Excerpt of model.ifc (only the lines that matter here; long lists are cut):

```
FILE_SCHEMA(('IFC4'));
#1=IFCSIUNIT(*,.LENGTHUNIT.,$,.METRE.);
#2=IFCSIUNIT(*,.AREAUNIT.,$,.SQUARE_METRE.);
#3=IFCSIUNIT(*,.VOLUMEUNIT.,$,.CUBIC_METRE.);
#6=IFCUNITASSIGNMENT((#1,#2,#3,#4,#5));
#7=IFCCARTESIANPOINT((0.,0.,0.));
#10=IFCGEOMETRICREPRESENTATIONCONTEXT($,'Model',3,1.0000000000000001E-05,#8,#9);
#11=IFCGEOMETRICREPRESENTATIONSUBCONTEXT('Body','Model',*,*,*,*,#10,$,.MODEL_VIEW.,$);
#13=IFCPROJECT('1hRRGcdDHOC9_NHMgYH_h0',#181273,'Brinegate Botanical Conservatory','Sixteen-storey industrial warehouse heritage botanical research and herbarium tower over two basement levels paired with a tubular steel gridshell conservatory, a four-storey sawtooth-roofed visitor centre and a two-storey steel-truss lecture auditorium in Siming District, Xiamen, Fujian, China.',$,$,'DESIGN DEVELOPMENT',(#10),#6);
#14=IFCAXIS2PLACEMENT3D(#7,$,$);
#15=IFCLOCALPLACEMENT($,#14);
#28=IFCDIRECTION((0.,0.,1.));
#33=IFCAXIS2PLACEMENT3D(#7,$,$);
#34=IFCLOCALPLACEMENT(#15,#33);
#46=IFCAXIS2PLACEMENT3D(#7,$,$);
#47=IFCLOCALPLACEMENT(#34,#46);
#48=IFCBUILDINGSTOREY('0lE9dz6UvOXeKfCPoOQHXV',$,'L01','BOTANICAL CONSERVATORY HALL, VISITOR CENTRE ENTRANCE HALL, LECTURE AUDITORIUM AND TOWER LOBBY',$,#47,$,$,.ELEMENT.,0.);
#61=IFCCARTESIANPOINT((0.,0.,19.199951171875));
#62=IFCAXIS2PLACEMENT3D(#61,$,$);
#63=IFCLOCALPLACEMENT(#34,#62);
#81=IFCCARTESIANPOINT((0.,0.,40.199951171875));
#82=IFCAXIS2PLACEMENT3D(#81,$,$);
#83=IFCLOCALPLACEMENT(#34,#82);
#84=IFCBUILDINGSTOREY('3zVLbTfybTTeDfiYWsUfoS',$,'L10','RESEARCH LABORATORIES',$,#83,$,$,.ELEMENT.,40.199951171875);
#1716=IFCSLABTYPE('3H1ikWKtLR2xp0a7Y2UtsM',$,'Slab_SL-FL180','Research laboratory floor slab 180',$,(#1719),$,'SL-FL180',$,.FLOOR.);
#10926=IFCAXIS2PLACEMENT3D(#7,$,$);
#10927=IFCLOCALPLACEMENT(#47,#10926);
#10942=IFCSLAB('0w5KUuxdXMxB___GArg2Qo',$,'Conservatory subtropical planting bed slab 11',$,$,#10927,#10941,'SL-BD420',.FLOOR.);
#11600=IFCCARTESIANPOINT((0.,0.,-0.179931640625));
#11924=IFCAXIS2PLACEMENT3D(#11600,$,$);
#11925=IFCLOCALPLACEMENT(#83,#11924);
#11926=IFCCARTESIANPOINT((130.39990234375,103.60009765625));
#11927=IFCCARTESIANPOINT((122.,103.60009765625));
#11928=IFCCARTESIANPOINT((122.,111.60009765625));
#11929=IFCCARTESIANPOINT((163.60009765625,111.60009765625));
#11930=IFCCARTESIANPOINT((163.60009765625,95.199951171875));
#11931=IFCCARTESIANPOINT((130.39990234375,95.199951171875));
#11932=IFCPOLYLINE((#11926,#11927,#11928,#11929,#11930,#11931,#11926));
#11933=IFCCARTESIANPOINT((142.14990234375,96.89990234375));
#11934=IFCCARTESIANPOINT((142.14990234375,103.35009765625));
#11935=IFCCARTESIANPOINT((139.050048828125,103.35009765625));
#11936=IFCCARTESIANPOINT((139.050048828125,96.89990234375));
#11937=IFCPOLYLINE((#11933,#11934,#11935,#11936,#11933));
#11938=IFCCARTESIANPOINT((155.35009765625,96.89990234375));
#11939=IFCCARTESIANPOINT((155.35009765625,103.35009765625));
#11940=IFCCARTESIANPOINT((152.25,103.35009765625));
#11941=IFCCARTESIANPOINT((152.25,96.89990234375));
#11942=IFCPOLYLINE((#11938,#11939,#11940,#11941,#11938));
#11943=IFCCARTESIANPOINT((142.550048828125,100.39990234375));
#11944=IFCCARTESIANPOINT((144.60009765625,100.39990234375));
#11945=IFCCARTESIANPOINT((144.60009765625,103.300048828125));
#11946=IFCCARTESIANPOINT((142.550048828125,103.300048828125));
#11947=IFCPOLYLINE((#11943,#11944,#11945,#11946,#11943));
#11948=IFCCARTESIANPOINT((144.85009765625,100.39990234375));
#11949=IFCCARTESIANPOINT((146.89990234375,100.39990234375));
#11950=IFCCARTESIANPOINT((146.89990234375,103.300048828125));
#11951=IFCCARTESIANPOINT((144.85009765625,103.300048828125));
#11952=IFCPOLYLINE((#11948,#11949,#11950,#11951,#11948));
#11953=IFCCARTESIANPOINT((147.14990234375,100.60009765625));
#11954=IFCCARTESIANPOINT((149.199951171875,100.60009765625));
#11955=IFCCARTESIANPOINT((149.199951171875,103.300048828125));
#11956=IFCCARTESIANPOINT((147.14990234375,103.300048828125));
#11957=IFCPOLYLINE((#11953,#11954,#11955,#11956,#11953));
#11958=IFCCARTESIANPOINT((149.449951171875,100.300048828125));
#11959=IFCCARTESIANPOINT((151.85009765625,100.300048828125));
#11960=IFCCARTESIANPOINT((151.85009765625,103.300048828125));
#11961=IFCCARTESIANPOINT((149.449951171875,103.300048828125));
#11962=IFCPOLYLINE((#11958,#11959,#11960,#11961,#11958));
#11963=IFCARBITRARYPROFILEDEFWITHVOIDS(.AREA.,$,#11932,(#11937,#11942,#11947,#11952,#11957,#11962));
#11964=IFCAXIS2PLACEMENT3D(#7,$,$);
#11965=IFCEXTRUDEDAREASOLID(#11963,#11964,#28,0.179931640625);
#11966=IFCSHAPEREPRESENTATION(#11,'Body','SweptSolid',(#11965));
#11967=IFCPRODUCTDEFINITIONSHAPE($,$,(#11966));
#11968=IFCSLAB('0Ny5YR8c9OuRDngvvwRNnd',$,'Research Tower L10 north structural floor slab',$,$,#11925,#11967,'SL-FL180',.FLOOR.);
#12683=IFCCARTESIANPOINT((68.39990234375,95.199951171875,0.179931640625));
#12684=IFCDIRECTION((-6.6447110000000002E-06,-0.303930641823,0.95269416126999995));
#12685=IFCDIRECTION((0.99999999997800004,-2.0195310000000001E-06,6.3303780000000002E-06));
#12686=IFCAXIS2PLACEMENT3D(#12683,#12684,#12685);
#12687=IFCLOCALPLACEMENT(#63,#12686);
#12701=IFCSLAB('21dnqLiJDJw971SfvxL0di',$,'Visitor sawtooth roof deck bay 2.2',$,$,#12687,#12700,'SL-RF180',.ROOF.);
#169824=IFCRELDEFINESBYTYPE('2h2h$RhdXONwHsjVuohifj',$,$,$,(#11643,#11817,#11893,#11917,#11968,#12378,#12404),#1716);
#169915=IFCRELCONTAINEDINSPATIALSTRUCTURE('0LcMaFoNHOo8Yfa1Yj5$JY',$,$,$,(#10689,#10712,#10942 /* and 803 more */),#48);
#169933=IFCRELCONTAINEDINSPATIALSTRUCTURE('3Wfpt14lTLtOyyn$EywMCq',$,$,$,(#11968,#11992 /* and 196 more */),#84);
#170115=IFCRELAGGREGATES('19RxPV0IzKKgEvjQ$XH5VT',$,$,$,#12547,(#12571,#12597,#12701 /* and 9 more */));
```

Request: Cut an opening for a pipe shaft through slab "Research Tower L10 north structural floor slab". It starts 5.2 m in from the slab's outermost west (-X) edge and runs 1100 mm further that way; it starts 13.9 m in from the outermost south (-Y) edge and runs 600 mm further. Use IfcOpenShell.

```python
import numpy as np
import ifcopenshell
import ifcopenshell.api.feature
import ifcopenshell.api.geometry
import ifcopenshell.api.root
import ifcopenshell.geom
import ifcopenshell.util.placement
import ifcopenshell.util.representation
import ifcopenshell.util.shape
import ifcopenshell.util.unit

model = ifcopenshell.open("model.ifc")
unit_scale = ifcopenshell.util.unit.calculate_unit_scale(model)
settings = ifcopenshell.geom.settings()


def volume(element):
    """Net volume in cubic metres, openings subtracted."""
    shape = ifcopenshell.geom.create_shape(settings, element)
    return ifcopenshell.util.shape.get_volume(shape.geometry)


slab = model.by_guid("0Ny5YR8c9OuRDngvvwRNnd")
before = volume(slab)

# Extent in the slab's own axes, in metres. The edges named are its -X and -Y sides.
slab_shape = ifcopenshell.geom.create_shape(settings, slab)
vertices = ifcopenshell.util.shape.get_vertices(slab_shape.geometry)
x_min, y_min, bottom = vertices.min(axis=0)
top = vertices[:, 2].max()

opening = ifcopenshell.api.root.create_entity(model, ifc_class="IfcOpeningElement", name="Pipe shaft opening", predefined_type="OPENING")
context = ifcopenshell.util.representation.get_context(model, "Model", "Body", "MODEL_VIEW")
width, depth = 1.1, 0.6
outline = [(0.0, 0.0), (width, 0.0), (width, depth), (0.0, depth), (0.0, 0.0)]
# Overshoot both faces by 50 mm so the cut is clean.
shape = ifcopenshell.api.geometry.add_slab_representation(
    model, context=context, depth=top - bottom + 0.1, polyline=outline
)
ifcopenshell.api.geometry.assign_representation(model, product=opening, representation=shape)

matrix = ifcopenshell.util.placement.get_local_placement(slab.ObjectPlacement)
matrix[:, 3] = matrix @ np.append(np.array([x_min + 5.2, y_min + 13.9, bottom - 0.05]) / unit_scale, 1.0)
ifcopenshell.api.geometry.edit_object_placement(model, product=opening, matrix=matrix, is_si=False)
ifcopenshell.api.feature.add_feature(model, feature=opening, element=slab)

after = volume(slab)

print(f"slab volume {before:.3f} -> {after:.3f} m3")

model.write("model_edited.ifc")
```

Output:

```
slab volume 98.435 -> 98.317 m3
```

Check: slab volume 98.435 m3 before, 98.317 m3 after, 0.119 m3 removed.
